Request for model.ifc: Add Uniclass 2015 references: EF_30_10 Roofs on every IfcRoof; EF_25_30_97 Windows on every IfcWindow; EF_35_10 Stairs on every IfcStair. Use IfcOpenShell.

First a look at what the model holds.

```python
import ifcopenshell

model = ifcopenshell.open("model.ifc")
print(model.schema)
print("classifications:", [c.Name for c in model.by_type("IfcClassification")])
for ifc_class in ("IfcDoor", "IfcRoof", "IfcStair", "IfcWall", "IfcWindow"):
    print(ifc_class, len(model.by_type(ifc_class)))
```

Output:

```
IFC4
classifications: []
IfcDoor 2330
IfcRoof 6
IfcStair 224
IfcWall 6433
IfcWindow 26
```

```python
import ifcopenshell
import ifcopenshell.api.classification

model = ifcopenshell.open("model.ifc")

system = ifcopenshell.api.classification.add_classification(model, classification="Uniclass 2015")

codes = {
    "IfcRoof": ("EF_30_10", "Roofs"),
    "IfcWindow": ("EF_25_30_97", "Windows"),
    "IfcStair": ("EF_35_10", "Stairs"),
}
for ifc_class, (code, name) in codes.items():
    products = model.by_type(ifc_class)
    ifcopenshell.api.classification.add_reference(
        model, products=products, classification=system, identification=code, name=name
    )
    print(code, len(products))

model.write("model_v2.ifc")
```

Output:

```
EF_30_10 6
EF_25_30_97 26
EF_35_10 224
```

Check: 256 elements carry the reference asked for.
